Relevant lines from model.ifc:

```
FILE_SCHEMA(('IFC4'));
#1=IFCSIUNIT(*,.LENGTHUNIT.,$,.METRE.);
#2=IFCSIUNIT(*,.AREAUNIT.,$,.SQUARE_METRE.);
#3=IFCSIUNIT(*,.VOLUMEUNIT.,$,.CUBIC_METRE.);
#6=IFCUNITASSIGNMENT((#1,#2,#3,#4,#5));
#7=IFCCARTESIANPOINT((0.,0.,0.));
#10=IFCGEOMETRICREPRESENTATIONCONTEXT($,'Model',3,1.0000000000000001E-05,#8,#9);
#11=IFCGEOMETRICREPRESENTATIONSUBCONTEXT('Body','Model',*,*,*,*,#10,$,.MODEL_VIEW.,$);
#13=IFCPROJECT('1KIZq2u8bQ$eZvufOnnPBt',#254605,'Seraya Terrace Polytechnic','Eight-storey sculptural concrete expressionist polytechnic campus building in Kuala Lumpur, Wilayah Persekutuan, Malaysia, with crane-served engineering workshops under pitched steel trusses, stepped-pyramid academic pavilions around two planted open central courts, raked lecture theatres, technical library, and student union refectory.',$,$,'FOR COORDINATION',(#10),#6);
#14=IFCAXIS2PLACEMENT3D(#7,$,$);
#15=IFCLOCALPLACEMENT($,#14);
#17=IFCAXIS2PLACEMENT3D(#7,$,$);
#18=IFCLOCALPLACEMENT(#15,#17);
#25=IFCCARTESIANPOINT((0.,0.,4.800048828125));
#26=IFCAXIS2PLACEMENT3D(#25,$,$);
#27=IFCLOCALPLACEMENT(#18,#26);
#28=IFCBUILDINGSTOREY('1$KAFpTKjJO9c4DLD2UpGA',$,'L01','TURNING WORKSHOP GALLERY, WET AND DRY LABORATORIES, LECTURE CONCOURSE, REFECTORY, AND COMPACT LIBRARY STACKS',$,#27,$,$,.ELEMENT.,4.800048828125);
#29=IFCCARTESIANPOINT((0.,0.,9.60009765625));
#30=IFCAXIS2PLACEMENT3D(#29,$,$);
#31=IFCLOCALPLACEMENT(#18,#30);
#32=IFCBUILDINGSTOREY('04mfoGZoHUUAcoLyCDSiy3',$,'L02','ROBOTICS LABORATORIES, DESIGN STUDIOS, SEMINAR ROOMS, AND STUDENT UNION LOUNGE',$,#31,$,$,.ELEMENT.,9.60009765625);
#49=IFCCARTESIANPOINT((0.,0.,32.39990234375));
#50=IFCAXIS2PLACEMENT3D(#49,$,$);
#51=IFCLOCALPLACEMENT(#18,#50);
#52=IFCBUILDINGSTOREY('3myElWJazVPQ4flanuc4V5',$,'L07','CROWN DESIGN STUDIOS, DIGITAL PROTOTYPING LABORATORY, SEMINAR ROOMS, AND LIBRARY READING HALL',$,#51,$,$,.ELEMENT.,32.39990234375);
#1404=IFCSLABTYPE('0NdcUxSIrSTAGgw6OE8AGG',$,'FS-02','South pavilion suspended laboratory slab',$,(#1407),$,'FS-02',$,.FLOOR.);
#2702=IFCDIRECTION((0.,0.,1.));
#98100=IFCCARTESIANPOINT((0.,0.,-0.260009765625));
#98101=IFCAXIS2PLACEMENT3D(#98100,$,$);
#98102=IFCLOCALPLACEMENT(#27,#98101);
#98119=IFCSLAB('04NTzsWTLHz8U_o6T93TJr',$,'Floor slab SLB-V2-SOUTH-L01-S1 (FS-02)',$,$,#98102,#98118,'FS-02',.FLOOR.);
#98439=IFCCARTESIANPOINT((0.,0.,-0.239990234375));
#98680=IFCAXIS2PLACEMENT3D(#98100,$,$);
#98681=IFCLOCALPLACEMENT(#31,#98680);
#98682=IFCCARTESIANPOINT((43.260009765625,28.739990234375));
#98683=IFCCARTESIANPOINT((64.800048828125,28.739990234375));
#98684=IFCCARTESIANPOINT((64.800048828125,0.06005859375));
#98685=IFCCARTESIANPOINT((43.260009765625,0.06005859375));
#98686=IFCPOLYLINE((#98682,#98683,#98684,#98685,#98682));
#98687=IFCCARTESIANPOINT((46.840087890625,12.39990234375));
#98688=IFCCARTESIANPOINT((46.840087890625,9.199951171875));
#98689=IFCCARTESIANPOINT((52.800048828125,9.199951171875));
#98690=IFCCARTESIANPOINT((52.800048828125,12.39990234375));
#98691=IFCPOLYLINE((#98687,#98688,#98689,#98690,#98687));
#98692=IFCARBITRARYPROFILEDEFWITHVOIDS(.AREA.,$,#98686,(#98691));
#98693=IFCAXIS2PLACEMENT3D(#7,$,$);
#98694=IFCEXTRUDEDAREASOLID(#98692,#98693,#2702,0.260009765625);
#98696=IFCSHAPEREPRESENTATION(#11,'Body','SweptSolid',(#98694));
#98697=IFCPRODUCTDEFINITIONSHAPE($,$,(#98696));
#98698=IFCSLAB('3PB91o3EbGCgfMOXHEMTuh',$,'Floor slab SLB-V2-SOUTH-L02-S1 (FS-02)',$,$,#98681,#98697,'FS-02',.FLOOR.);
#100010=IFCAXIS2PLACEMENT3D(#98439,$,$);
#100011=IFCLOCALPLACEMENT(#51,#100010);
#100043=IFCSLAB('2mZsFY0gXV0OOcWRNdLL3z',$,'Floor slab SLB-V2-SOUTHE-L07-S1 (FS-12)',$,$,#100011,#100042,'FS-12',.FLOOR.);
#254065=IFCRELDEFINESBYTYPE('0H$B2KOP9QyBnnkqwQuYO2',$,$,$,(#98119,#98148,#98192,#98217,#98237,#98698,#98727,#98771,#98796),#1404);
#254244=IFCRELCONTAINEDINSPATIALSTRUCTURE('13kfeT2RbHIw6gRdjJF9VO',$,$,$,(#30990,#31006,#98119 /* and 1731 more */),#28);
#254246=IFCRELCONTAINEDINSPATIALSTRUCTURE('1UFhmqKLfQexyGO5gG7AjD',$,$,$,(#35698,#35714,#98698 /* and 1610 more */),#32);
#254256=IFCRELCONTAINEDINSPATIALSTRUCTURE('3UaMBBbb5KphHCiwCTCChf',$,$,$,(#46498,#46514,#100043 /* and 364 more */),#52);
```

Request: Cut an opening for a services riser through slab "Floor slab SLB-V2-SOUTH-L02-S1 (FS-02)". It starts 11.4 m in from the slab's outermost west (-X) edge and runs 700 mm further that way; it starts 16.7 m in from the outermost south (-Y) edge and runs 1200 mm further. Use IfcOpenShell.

```python
import numpy as np
import ifcopenshell
import ifcopenshell.api.feature
import ifcopenshell.api.geometry
import ifcopenshell.api.root
import ifcopenshell.geom
import ifcopenshell.util.placement
import ifcopenshell.util.representation
import ifcopenshell.util.shape
import ifcopenshell.util.unit

model = ifcopenshell.open("model.ifc")
unit_scale = ifcopenshell.util.unit.calculate_unit_scale(model)
settings = ifcopenshell.geom.settings()


def volume(element):
    """Net volume in cubic metres, openings subtracted."""
    shape = ifcopenshell.geom.create_shape(settings, element)
    return ifcopenshell.util.shape.get_volume(shape.geometry)


slab = model.by_guid("3PB91o3EbGCgfMOXHEMTuh")
before = volume(slab)

# Extent in the slab's own axes, in metres. The edges named are its -X and -Y sides.
slab_shape = ifcopenshell.geom.create_shape(settings, slab)
vertices = ifcopenshell.util.shape.get_vertices(slab_shape.geometry)
x_min, y_min, bottom = vertices.min(axis=0)
top = vertices[:, 2].max()

opening = ifcopenshell.api.root.create_entity(model, ifc_class="IfcOpeningElement", name="Services riser opening", predefined_type="OPENING")
context = ifcopenshell.util.representation.get_context(model, "Model", "Body", "MODEL_VIEW")
width, depth = 0.7, 1.2
outline = [(0.0, 0.0), (width, 0.0), (width, depth), (0.0, depth), (0.0, 0.0)]
# Overshoot both faces by 50 mm so the cut is clean.
shape = ifcopenshell.api.geometry.add_slab_representation(
    model, context=context, depth=top - bottom + 0.1, polyline=outline
)
ifcopenshell.api.geometry.assign_representation(model, product=opening, representation=shape)

matrix = ifcopenshell.util.placement.get_local_placement(slab.ObjectPlacement)
matrix[:, 3] = matrix @ np.append(np.array([x_min + 11.4, y_min + 16.7, bottom - 0.05]) / unit_scale, 1.0)
ifcopenshell.api.geometry.edit_object_placement(model, product=opening, matrix=matrix, is_si=False)
ifcopenshell.api.feature.add_feature(model, feature=opening, element=slab)

after = volume(slab)

print(f"slab volume {before:.3f} -> {after:.3f} m3")

model.write("model_edited.ifc")
```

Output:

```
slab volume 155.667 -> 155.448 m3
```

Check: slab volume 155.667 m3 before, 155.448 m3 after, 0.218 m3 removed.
